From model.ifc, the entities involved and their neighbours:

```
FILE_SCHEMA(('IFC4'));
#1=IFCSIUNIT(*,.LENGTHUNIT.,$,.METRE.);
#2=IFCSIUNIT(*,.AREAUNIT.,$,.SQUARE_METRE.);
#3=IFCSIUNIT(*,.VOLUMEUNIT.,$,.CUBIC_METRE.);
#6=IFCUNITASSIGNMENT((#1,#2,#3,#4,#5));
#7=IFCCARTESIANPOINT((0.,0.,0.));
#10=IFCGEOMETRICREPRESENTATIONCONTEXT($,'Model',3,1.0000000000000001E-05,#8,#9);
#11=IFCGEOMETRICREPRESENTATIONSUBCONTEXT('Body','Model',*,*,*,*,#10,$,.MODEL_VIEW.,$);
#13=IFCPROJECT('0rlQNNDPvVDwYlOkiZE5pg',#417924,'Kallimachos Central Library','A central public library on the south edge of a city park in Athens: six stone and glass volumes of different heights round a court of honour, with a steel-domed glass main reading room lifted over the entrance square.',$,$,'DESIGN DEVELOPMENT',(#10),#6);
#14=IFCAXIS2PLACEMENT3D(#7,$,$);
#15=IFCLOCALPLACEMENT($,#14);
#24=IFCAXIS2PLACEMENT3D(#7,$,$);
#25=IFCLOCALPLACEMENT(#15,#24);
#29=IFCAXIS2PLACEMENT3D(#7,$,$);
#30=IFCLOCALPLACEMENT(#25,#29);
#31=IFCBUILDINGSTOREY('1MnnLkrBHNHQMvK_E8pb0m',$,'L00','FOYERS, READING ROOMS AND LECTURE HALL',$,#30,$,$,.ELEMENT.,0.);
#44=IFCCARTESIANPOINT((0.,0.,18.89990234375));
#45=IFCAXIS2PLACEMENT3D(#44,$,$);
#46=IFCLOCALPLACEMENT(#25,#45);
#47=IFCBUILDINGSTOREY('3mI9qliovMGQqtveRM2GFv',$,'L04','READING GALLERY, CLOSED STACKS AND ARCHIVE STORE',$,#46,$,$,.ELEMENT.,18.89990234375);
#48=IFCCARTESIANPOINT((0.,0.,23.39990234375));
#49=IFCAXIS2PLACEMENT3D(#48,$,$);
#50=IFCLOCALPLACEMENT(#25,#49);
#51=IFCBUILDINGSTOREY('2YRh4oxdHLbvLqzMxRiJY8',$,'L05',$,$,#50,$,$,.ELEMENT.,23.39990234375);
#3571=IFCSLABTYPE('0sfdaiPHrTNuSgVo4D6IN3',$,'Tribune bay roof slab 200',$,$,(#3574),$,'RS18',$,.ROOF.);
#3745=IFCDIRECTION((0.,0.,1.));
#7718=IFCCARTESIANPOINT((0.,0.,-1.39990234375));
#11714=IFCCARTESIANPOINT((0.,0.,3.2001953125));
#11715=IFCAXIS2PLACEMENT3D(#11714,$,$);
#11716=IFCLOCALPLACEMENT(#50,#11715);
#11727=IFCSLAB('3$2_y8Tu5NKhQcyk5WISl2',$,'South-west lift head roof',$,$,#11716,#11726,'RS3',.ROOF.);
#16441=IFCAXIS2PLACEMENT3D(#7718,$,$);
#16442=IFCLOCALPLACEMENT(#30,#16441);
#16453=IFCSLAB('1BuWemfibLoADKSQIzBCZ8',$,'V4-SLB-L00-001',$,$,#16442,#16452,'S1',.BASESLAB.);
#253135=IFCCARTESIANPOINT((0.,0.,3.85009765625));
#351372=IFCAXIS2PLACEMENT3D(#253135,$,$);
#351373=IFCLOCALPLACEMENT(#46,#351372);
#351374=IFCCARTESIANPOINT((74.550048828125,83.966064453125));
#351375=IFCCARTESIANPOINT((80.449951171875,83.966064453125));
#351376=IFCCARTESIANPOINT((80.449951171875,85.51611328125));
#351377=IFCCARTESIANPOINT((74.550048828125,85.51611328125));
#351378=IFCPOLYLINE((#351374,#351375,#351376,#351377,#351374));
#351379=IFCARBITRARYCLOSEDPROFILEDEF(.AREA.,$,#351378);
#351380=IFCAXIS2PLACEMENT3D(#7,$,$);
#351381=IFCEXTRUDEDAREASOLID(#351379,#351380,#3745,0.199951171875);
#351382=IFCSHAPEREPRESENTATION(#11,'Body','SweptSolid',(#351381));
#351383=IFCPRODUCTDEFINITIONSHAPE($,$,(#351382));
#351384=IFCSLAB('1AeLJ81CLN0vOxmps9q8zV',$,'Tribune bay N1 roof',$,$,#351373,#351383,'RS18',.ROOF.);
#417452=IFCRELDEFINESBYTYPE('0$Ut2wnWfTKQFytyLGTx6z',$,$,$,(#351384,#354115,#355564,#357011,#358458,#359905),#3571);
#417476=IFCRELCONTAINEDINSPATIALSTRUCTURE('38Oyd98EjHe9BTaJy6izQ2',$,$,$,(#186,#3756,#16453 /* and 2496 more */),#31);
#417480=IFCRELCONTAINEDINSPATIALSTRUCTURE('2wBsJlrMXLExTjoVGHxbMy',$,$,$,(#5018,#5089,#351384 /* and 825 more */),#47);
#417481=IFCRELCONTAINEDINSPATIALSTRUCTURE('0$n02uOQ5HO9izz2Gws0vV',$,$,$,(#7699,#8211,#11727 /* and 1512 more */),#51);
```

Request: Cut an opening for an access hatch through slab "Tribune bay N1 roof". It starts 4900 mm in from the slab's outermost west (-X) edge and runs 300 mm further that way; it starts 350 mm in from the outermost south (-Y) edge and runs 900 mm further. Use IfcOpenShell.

```python
import numpy as np
import ifcopenshell
import ifcopenshell.api.feature
import ifcopenshell.api.geometry
import ifcopenshell.api.root
import ifcopenshell.geom
import ifcopenshell.util.placement
import ifcopenshell.util.representation
import ifcopenshell.util.shape
import ifcopenshell.util.unit

model = ifcopenshell.open("model.ifc")
unit_scale = ifcopenshell.util.unit.calculate_unit_scale(model)
settings = ifcopenshell.geom.settings()


def volume(element):
    """Net volume in cubic metres, openings subtracted."""
    shape = ifcopenshell.geom.create_shape(settings, element)
    return ifcopenshell.util.shape.get_volume(shape.geometry)


slab = model.by_id(351384)
before = volume(slab)

# Extent in the slab's own axes, in metres. The edges named are its -X and -Y sides.
slab_shape = ifcopenshell.geom.create_shape(settings, slab)
vertices = ifcopenshell.util.shape.get_vertices(slab_shape.geometry)
x_min, y_min, bottom = vertices.min(axis=0)
top = vertices[:, 2].max()

opening = ifcopenshell.api.root.create_entity(model, ifc_class="IfcOpeningElement", name="Access hatch opening", predefined_type="OPENING")
context = ifcopenshell.util.representation.get_context(model, "Model", "Body", "MODEL_VIEW")
width, depth = 0.3, 0.9
outline = [(0.0, 0.0), (width, 0.0), (width, depth), (0.0, depth), (0.0, 0.0)]
# Overshoot both faces by 50 mm so the cut is clean.
shape = ifcopenshell.api.geometry.add_slab_representation(
    model, context=context, depth=top - bottom + 0.1, polyline=outline
)
ifcopenshell.api.geometry.assign_representation(model, product=opening, representation=shape)

matrix = ifcopenshell.util.placement.get_local_placement(slab.ObjectPlacement)
matrix[:, 3] = matrix @ np.append(np.array([x_min + 4.9, y_min + 0.35, bottom - 0.05]) / unit_scale, 1.0)
ifcopenshell.api.geometry.edit_object_placement(model, product=opening, matrix=matrix, is_si=False)
ifcopenshell.api.feature.add_feature(model, feature=opening, element=slab)

after = volume(slab)

print(f"slab volume {before:.3f} -> {after:.3f} m3")

model.write("model-out.ifc")
```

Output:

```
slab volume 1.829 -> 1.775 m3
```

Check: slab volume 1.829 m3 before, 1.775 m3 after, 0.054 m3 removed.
